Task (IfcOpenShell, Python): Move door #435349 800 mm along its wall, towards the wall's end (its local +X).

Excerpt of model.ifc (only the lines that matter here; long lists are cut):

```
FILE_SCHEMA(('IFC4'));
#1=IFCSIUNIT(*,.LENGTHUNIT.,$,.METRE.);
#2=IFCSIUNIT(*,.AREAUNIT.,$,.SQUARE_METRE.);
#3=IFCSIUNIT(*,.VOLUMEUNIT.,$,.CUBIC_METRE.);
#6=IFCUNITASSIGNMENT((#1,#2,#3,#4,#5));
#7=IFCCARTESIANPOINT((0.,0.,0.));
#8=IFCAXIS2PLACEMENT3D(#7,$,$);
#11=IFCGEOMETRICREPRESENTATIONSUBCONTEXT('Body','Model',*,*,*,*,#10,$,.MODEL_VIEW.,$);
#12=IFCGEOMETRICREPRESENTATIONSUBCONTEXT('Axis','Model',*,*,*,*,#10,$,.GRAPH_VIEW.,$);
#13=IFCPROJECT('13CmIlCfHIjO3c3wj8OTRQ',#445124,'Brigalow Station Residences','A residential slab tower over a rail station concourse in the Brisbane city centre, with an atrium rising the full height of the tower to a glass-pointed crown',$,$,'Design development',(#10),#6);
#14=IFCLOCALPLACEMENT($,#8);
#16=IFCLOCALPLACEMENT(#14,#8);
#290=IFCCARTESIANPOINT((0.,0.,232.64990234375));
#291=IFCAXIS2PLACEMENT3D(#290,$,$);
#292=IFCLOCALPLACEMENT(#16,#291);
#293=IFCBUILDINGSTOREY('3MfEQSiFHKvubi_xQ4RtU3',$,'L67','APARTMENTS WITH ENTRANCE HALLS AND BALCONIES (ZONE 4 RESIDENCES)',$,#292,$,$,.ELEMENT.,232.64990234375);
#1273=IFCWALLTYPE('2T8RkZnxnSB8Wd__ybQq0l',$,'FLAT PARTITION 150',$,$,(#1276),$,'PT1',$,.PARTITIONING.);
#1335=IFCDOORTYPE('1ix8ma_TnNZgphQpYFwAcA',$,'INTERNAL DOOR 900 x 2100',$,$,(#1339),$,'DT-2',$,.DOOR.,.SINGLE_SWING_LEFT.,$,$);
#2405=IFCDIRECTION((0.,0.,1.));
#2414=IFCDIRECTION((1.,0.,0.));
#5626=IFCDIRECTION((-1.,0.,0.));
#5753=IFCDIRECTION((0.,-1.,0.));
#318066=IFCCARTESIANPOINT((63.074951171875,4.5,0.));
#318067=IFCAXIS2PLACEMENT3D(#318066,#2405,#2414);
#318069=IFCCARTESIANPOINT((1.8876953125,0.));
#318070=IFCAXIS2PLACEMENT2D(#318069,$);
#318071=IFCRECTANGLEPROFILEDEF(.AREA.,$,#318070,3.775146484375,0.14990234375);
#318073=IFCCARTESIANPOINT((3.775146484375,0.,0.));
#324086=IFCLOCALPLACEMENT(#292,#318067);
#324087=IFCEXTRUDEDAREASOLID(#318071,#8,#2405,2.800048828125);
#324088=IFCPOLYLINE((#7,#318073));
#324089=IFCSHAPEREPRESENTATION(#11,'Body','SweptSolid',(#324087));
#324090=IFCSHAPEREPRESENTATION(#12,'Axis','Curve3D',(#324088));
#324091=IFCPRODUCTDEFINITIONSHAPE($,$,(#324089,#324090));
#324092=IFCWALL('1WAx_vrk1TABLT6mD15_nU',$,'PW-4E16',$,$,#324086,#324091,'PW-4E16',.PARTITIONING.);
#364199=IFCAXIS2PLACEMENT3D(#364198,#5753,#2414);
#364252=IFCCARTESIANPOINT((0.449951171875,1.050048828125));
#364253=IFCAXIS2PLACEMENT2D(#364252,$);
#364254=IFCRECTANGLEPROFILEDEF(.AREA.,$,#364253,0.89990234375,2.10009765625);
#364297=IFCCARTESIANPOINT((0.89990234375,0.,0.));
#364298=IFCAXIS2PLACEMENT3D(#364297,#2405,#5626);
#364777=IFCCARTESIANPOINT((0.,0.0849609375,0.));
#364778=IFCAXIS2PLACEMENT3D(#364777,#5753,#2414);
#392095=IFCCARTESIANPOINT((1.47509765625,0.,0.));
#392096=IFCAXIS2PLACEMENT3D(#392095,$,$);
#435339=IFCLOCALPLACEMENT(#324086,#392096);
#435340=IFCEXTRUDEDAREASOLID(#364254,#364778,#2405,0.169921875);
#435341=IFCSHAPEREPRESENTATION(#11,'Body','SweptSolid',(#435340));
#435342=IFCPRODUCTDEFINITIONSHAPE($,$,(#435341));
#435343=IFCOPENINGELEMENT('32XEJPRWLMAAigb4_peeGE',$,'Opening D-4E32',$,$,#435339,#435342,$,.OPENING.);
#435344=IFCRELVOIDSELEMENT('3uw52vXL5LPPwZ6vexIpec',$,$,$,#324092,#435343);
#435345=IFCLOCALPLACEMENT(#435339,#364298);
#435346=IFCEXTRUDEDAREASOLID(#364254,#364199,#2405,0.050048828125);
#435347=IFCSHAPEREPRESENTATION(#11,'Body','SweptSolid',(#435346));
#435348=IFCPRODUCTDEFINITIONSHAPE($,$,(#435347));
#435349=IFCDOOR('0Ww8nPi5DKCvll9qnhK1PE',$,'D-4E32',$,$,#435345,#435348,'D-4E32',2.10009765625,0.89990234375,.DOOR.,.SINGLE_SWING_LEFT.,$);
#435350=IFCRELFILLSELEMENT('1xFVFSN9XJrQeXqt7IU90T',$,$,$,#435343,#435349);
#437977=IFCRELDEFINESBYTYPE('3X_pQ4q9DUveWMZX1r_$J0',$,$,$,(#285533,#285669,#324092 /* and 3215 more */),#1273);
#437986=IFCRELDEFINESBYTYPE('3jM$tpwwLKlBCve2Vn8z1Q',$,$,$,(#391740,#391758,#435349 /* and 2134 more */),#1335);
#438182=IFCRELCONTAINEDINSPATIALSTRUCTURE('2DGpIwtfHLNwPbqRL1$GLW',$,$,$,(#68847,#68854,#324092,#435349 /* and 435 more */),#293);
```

```python
import ifcopenshell
import ifcopenshell.api.geometry
import ifcopenshell.util.placement

model = ifcopenshell.open("model.ifc")

door = model.by_guid("0Ww8nPi5DKCvll9qnhK1PE")
opening = door.FillsVoids[0].RelatingOpeningElement
wall = opening.VoidsElements[0].RelatingBuildingElement

wall_matrix = ifcopenshell.util.placement.get_local_placement(wall.ObjectPlacement)
shift = wall_matrix[:3, 0] * 0.8
before = ifcopenshell.util.placement.get_local_placement(door.ObjectPlacement)[:3, 3].copy()

# The door is placed relative to its opening, so it follows when the opening moves.
matrix = ifcopenshell.util.placement.get_local_placement(opening.ObjectPlacement)
matrix[:3, 3] += shift
ifcopenshell.api.geometry.edit_object_placement(
    model, product=opening, matrix=matrix, is_si=False, should_transform_children=True
)

after = ifcopenshell.util.placement.get_local_placement(door.ObjectPlacement)[:3, 3]
print("door moved by", (after - before).round(3) + 0.0)

model.write("model_updated.ifc")
```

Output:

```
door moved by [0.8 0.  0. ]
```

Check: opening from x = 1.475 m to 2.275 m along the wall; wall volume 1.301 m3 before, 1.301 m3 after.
